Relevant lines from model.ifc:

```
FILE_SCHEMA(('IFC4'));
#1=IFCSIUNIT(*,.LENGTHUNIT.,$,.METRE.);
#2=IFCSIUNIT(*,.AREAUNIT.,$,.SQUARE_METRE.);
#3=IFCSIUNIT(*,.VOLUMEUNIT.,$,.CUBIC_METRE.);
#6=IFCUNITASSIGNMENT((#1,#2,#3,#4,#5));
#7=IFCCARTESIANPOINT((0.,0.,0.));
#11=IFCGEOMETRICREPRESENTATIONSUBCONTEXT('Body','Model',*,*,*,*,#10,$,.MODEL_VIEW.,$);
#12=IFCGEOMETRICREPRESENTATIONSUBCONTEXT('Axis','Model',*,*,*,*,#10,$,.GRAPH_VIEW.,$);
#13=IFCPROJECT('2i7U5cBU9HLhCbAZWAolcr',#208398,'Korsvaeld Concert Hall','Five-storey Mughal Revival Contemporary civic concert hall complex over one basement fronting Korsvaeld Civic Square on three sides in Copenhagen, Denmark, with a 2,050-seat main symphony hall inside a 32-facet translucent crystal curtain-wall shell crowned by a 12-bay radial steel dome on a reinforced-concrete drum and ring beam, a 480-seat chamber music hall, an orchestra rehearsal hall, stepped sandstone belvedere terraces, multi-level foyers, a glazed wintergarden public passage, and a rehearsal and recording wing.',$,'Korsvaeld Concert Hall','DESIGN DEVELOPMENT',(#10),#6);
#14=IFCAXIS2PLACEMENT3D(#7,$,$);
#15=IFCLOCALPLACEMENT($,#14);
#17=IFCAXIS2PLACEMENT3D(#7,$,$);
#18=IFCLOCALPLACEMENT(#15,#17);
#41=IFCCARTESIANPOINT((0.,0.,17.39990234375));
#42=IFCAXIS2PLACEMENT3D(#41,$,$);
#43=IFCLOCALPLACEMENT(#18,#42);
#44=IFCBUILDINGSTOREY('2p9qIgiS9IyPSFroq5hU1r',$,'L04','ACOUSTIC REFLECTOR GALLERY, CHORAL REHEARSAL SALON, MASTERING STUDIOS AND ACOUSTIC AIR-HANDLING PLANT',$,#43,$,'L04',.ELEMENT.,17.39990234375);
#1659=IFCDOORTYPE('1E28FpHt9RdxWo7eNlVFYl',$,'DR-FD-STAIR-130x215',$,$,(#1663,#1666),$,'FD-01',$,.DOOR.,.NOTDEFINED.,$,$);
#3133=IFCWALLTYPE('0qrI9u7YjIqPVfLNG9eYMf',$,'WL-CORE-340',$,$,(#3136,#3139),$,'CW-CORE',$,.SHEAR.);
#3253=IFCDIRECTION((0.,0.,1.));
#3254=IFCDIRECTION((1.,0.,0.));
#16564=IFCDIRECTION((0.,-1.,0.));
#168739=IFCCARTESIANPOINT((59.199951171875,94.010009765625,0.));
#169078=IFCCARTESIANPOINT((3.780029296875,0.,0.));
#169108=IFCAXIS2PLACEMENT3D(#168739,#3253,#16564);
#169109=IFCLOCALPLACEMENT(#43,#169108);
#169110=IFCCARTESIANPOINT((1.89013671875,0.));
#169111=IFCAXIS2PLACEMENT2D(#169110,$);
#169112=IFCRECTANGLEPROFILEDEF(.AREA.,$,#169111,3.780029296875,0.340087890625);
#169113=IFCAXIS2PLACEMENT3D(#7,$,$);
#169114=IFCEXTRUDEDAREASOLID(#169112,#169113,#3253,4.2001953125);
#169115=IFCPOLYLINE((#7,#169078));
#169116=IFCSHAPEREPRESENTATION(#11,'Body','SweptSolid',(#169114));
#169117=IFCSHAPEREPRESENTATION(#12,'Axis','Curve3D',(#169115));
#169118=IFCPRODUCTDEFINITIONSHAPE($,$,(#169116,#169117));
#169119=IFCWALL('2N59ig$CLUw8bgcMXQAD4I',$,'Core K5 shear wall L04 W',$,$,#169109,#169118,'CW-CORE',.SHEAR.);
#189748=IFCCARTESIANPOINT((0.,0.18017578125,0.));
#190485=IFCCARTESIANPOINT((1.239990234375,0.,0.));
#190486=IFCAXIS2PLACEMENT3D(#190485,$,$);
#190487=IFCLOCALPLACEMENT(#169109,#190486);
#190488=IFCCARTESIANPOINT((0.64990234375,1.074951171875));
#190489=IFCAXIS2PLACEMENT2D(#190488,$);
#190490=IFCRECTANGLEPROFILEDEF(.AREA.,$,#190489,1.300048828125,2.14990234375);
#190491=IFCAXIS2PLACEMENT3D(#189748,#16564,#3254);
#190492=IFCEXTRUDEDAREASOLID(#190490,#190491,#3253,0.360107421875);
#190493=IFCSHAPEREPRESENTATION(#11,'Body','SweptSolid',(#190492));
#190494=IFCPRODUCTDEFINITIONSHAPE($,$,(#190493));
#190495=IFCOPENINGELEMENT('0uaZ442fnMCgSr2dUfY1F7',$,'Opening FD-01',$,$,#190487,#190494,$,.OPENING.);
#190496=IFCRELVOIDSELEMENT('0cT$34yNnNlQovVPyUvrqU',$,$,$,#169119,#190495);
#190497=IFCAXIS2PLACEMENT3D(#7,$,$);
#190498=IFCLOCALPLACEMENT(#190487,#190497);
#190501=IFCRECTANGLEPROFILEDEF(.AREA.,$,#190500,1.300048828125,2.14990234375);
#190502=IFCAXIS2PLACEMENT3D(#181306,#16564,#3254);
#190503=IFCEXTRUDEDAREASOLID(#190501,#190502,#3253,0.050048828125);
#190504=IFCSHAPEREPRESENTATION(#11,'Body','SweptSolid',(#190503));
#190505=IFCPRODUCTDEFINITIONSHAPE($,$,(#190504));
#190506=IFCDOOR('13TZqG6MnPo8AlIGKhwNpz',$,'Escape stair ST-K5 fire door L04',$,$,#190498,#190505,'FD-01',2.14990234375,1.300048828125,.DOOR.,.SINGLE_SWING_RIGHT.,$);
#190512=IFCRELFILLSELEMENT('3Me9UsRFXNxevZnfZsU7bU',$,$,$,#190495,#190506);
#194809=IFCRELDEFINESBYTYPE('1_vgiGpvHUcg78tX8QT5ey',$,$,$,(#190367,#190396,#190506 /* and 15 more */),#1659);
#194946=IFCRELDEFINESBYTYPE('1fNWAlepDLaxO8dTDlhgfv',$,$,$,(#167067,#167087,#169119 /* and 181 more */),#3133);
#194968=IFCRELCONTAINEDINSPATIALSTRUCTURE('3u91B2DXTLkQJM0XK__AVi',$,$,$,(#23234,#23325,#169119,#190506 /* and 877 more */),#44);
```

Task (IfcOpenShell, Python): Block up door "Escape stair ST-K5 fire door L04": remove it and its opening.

```python
import ifcopenshell
import ifcopenshell.api.feature
import ifcopenshell.api.root
import ifcopenshell.geom
import ifcopenshell.util.shape

model = ifcopenshell.open("model.ifc")
settings = ifcopenshell.geom.settings()


def volume(element):
    """Net volume in cubic metres, openings subtracted."""
    shape = ifcopenshell.geom.create_shape(settings, element)
    return ifcopenshell.util.shape.get_volume(shape.geometry)


door = model.by_guid("13TZqG6MnPo8AlIGKhwNpz")
opening = door.FillsVoids[0].RelatingOpeningElement
wall = opening.VoidsElements[0].RelatingBuildingElement
before = volume(wall)

ifcopenshell.api.root.remove_product(model, product=door)
ifcopenshell.api.feature.remove_feature(model, feature=opening)

after = volume(wall)

print(f"wall volume {before:.3f} -> {after:.3f} m3")

model.write("model_v2.ifc")
```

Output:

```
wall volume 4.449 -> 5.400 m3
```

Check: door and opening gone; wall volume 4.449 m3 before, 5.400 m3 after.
